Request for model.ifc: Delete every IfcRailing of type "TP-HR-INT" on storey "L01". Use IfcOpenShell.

First a look at what the model holds.

```python
import ifcopenshell
import ifcopenshell.util.element

model = ifcopenshell.open("model.ifc")
print(model.schema)
storey = next(s for s in model.by_type("IfcBuildingStorey") if s.Name == "L01")
railings = [e for e in ifcopenshell.util.element.get_decomposition(storey) if e.is_a("IfcRailing")]
seen = {}
for e in railings:
    element_type = ifcopenshell.util.element.get_type(e)
    name = element_type.Name if element_type not in (None, e) else None
    seen[name] = seen.get(name, 0) + 1
for name, count in sorted(seen.items(), key=str):
    print(count, "x", name)
```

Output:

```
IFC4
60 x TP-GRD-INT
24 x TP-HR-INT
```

```python
import ifcopenshell
import ifcopenshell.api.root
import ifcopenshell.util.element

model = ifcopenshell.open("model.ifc")

storey = next(s for s in model.by_type("IfcBuildingStorey") if s.Name == "L01")
railings = [e for e in ifcopenshell.util.element.get_decomposition(storey) if e.is_a("IfcRailing")]
targets = [e for e in railings if (t := ifcopenshell.util.element.get_type(e)) not in (None, e) and t.Name == "TP-HR-INT"]

for e in targets:
    ifcopenshell.api.root.remove_product(model, product=e)
print(len(targets), "removed")

model.write("model-out.ifc")
```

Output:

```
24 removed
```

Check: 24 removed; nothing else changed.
